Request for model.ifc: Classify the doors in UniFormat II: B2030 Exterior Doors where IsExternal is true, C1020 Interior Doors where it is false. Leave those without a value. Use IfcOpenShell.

First a look at what the model holds.

```python
import ifcopenshell
import ifcopenshell.util.element

model = ifcopenshell.open("model.ifc")
print(model.schema)
print("classifications:", [c.Name for c in model.by_type("IfcClassification")])
values = [ifcopenshell.util.element.get_pset(e, "Pset_DoorCommon", "IsExternal") for e in model.by_type("IfcDoor")]
for value in (True, False, None):
    print("IsExternal", value, values.count(value))
```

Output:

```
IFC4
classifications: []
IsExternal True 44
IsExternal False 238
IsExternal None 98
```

```python
import ifcopenshell
import ifcopenshell.api.classification
import ifcopenshell.util.element

model = ifcopenshell.open("model.ifc")

system = ifcopenshell.api.classification.add_classification(model, classification="UniFormat II")

doors = model.by_type("IfcDoor")
external = {e: ifcopenshell.util.element.get_pset(e, "Pset_DoorCommon", "IsExternal") for e in doors}
for flag, code, name in ((True, "B2030", "Exterior Doors"), (False, "C1020", "Interior Doors")):
    products = [e for e in doors if external[e] is flag]
    ifcopenshell.api.classification.add_reference(
        model, products=products, classification=system, identification=code, name=name
    )
    print(code, len(products))

model.write("model_updated.ifc")
```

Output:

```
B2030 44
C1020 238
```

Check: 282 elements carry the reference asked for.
